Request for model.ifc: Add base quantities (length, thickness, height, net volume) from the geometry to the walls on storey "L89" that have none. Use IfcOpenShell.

First a look at what the model holds.

```python
import ifcopenshell
import ifcopenshell.util.element
import ifcopenshell.util.unit

model = ifcopenshell.open("model.ifc")
print(model.schema)
for unit_type in ("LENGTHUNIT", "AREAUNIT", "VOLUMEUNIT"):
    print(unit_type, ifcopenshell.util.unit.calculate_unit_scale(model, unit_type))
storey = next(s for s in model.by_type("IfcBuildingStorey") if s.Name == "L89")
walls = [e for e in ifcopenshell.util.element.get_decomposition(storey) if e.is_a("IfcWall")]
for e in sorted(walls, key=lambda e: e.id()):
    print(e.id(), e.is_a(), e.Name, list(ifcopenshell.util.element.get_psets(e, qtos_only=True)), sep=" | ")
```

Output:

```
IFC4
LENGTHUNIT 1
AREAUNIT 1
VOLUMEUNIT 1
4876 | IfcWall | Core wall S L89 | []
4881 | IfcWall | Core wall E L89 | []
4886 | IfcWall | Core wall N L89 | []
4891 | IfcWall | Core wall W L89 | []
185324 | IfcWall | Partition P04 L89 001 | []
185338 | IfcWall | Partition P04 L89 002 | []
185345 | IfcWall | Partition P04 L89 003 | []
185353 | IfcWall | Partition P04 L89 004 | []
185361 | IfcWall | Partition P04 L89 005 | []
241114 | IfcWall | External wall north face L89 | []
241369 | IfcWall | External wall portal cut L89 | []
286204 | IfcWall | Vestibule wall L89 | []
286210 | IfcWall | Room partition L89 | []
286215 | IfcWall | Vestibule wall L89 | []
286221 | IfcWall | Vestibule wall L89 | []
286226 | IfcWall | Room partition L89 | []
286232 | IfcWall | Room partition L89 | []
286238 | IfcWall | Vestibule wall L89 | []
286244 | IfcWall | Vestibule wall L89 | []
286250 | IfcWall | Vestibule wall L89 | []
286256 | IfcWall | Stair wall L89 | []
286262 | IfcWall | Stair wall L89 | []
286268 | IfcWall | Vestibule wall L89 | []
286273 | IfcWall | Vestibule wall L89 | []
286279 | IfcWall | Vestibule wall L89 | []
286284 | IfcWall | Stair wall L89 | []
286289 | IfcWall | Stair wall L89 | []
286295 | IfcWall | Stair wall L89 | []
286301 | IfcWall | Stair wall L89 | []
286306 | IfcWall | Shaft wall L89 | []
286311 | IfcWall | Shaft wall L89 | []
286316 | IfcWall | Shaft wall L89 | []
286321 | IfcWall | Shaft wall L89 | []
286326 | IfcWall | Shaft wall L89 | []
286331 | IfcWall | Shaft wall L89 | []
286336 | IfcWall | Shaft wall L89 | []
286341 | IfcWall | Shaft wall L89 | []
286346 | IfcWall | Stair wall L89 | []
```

```python
import ifcopenshell
import ifcopenshell.api.pset
import ifcopenshell.geom
import ifcopenshell.util.element
import ifcopenshell.util.shape
import ifcopenshell.util.unit

model = ifcopenshell.open("model.ifc")
unit_scale = ifcopenshell.util.unit.calculate_unit_scale(model)
volume_scale = ifcopenshell.util.unit.calculate_unit_scale(model, "VOLUMEUNIT")
settings = ifcopenshell.geom.settings()

storey = next(s for s in model.by_type("IfcBuildingStorey") if s.Name == "L89")
walls = [e for e in ifcopenshell.util.element.get_decomposition(storey) if e.is_a("IfcWall")]

for e in sorted(walls, key=lambda e: e.id()):
    if ifcopenshell.util.element.get_psets(e, qtos_only=True, should_inherit=False):
        continue
    # Geometry comes back in metres, in the element's own axes.
    shape = ifcopenshell.geom.create_shape(settings, e)
    values = {
        "Length": ifcopenshell.util.shape.get_x(shape.geometry) / unit_scale,
        "Width": ifcopenshell.util.shape.get_y(shape.geometry) / unit_scale,
        "Height": ifcopenshell.util.shape.get_z(shape.geometry) / unit_scale,
        "NetVolume": ifcopenshell.util.shape.get_volume(shape.geometry) / volume_scale,
    }
    qto = ifcopenshell.api.pset.add_qto(model, product=e, name="Qto_WallBaseQuantities")
    ifcopenshell.api.pset.edit_qto(model, qto=qto, properties=values)
    print(e.id(), {k: round(v, 3) for k, v in values.items()})

model.write("model_rev.ifc")
```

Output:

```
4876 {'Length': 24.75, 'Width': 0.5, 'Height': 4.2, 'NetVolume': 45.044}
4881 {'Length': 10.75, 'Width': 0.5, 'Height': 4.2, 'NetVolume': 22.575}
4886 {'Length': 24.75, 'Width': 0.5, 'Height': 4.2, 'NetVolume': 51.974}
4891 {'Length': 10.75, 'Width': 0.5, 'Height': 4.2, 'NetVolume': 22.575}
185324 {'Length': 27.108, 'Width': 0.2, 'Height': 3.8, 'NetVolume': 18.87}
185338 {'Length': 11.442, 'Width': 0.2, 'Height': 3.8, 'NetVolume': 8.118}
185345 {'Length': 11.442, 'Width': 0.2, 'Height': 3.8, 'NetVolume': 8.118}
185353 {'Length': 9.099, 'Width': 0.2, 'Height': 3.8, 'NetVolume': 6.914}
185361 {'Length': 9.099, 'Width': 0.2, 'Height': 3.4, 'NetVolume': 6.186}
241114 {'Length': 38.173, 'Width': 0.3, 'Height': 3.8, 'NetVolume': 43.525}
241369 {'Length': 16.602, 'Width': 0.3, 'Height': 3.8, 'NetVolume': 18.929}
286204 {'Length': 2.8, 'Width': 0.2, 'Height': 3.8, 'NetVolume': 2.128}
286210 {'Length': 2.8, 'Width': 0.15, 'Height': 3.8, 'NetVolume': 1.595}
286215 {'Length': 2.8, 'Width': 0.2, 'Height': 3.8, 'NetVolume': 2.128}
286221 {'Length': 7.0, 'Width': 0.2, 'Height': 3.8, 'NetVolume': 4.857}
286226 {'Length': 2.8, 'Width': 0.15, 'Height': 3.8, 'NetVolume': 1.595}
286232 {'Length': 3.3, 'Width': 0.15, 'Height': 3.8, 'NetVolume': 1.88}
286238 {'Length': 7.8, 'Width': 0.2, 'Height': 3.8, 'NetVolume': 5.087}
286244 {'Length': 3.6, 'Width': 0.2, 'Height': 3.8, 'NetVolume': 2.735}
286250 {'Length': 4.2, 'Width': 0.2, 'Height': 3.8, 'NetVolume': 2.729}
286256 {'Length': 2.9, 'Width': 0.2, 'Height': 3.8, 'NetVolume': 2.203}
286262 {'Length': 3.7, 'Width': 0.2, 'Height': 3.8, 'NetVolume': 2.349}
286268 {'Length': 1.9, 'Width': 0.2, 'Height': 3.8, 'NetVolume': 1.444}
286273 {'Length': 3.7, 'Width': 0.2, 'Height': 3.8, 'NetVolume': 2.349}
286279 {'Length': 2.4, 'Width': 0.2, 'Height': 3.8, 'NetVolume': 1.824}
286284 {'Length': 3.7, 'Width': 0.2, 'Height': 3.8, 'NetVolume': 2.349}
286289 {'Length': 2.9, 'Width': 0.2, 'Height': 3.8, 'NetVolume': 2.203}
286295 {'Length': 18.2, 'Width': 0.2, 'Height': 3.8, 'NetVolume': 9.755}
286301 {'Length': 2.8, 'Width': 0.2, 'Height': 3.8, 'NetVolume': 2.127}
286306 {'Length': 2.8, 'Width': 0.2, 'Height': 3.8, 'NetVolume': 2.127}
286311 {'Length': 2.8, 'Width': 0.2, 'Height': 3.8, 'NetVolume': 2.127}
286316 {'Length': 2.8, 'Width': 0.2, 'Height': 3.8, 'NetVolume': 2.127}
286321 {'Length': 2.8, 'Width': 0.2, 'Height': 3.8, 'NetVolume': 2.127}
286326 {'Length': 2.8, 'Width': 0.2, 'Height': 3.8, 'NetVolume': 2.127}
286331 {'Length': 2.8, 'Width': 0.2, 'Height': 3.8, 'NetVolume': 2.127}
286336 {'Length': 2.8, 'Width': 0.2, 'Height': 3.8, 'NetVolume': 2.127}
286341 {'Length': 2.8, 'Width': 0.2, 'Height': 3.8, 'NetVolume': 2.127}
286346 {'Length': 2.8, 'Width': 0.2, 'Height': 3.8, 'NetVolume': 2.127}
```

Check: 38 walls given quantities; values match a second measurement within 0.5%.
